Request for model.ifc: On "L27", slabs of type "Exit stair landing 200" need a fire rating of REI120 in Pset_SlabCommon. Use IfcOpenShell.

First a look at what the model holds.

```python
import ifcopenshell
import ifcopenshell.util.element

model = ifcopenshell.open("model.ifc")
print(model.schema)
storey = next(s for s in model.by_type("IfcBuildingStorey") if s.Name == "L27")
slabs = [e for e in ifcopenshell.util.element.get_decomposition(storey) if e.is_a("IfcSlab")]
seen = {}
for e in slabs:
    element_type = ifcopenshell.util.element.get_type(e)
    key = (element_type.Name if element_type != e and element_type else None, ifcopenshell.util.element.get_pset(e, "Pset_SlabCommon", "FireRating"))
    seen[key] = seen.get(key, 0) + 1
for (name, value), count in sorted(seen.items(), key=str):
    print(count, "x", name, "|", value)
```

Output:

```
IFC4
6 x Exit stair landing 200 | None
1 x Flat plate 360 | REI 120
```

```python
import ifcopenshell
import ifcopenshell.api.pset
import ifcopenshell.util.element

model = ifcopenshell.open("model.ifc")

storey = next(s for s in model.by_type("IfcBuildingStorey") if s.Name == "L27")
slabs = [e for e in ifcopenshell.util.element.get_decomposition(storey) if e.is_a("IfcSlab")]

count = 0
for e in slabs:
    element_type = ifcopenshell.util.element.get_type(e)
    if element_type in (None, e) or element_type.Name != "Exit stair landing 200":
        continue
    found = ifcopenshell.util.element.get_pset(e, "Pset_SlabCommon", should_inherit=False)
    if found:
        pset = model.by_id(found["id"])
        if len(ifcopenshell.util.element.get_elements_by_pset(pset)) > 1:
            pset = ifcopenshell.api.pset.unshare_pset(model, products=[e], pset=pset)[0]
    else:
        pset = ifcopenshell.api.pset.add_pset(model, product=e, name="Pset_SlabCommon")
    ifcopenshell.api.pset.edit_pset(model, pset=pset, properties={"FireRating": "REI120"})
    count += 1

print(count, "slabs updated")

model.write("model-out.ifc")
```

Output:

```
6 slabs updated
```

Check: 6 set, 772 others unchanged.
